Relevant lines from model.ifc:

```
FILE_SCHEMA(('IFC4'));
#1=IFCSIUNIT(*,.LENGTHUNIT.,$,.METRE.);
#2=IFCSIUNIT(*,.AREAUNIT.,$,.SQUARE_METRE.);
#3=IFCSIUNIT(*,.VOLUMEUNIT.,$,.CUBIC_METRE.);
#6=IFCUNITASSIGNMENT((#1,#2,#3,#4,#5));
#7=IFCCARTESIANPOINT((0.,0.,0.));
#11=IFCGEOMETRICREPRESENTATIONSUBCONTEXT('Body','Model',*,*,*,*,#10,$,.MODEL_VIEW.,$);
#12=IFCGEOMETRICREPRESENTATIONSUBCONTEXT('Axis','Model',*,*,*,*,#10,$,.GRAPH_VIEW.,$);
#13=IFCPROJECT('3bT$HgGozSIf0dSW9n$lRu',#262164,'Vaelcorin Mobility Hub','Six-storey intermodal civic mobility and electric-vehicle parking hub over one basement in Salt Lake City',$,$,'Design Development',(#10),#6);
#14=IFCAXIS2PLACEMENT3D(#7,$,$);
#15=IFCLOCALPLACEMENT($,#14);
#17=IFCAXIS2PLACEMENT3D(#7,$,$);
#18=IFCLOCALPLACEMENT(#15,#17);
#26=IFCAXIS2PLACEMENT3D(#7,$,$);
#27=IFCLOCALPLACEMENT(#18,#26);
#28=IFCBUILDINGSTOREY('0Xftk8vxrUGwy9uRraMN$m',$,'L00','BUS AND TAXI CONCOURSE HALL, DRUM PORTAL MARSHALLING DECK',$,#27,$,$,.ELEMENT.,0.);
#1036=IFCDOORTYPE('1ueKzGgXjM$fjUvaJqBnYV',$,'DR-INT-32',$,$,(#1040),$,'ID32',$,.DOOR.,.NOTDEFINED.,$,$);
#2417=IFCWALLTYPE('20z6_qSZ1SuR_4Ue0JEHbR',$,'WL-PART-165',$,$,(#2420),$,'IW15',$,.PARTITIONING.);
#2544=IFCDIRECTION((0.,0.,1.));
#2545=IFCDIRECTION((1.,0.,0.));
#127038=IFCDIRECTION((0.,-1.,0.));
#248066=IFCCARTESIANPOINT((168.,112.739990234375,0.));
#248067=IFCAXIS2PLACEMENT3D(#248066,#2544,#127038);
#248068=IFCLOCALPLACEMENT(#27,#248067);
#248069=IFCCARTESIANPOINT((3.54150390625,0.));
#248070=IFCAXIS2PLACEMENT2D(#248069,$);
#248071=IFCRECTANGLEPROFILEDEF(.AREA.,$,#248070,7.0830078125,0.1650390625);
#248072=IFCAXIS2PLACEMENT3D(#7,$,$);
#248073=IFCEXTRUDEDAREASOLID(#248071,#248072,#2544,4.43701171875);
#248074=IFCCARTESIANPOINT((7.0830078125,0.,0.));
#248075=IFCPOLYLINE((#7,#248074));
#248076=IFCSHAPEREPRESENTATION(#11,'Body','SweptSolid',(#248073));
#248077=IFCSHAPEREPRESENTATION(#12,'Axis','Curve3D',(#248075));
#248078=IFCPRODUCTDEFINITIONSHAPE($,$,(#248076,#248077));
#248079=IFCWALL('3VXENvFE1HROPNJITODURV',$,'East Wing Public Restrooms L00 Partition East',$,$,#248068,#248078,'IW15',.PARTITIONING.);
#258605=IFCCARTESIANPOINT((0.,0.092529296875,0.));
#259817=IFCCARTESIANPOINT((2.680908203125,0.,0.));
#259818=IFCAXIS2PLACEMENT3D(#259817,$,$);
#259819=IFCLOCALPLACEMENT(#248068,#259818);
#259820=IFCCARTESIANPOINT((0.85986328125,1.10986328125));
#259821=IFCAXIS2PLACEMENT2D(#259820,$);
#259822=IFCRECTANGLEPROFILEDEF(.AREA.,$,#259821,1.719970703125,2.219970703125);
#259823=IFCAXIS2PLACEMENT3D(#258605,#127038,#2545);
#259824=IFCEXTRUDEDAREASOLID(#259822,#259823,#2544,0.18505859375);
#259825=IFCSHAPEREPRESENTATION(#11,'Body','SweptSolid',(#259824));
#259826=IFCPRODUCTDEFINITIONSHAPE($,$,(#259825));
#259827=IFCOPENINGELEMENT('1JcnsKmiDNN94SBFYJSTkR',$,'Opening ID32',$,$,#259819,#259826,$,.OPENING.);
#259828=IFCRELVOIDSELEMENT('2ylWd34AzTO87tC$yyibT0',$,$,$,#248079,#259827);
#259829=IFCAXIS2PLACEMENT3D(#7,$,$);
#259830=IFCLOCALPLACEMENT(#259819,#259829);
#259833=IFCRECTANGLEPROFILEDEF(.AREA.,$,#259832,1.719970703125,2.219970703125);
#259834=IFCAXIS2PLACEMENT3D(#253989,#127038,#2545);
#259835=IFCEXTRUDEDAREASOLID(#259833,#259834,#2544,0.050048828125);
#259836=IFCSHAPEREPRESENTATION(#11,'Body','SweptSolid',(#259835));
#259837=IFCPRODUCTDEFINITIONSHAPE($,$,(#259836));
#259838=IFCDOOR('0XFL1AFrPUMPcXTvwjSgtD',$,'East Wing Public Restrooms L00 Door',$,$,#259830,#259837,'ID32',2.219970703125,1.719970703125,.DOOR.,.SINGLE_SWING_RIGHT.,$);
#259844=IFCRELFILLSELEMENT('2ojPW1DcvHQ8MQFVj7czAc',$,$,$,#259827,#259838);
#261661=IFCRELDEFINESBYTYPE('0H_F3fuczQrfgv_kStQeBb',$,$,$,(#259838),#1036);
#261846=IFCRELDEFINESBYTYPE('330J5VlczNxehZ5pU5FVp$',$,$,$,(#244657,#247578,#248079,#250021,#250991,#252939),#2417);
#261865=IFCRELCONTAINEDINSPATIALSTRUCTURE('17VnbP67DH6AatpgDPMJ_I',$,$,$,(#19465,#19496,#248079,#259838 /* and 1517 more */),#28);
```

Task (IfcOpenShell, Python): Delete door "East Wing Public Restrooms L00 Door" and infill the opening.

```python
import ifcopenshell
import ifcopenshell.api.feature
import ifcopenshell.api.root
import ifcopenshell.geom
import ifcopenshell.util.shape

model = ifcopenshell.open("model.ifc")
settings = ifcopenshell.geom.settings()


def volume(element):
    """Net volume in cubic metres, openings subtracted."""
    shape = ifcopenshell.geom.create_shape(settings, element)
    return ifcopenshell.util.shape.get_volume(shape.geometry)


door = model.by_guid("0XFL1AFrPUMPcXTvwjSgtD")
opening = door.FillsVoids[0].RelatingOpeningElement
wall = opening.VoidsElements[0].RelatingBuildingElement
before = volume(wall)

ifcopenshell.api.root.remove_product(model, product=door)
ifcopenshell.api.feature.remove_feature(model, feature=opening)

after = volume(wall)

print(f"wall volume {before:.3f} -> {after:.3f} m3")

model.write("model_updated.ifc")
```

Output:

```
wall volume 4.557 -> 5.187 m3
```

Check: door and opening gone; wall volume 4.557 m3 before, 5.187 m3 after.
